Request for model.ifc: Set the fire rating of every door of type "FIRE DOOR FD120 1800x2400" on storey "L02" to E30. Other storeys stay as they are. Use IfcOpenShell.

First a look at what the model holds.

```python
import ifcopenshell
import ifcopenshell.util.element

model = ifcopenshell.open("model.ifc")
print(model.schema)
storey = next(s for s in model.by_type("IfcBuildingStorey") if s.Name == "L02")
doors = [e for e in ifcopenshell.util.element.get_decomposition(storey) if e.is_a("IfcDoor")]
seen = {}
for e in doors:
    element_type = ifcopenshell.util.element.get_type(e)
    key = (element_type.Name if element_type != e and element_type else None, ifcopenshell.util.element.get_pset(e, "Pset_DoorCommon", "FireRating"))
    seen[key] = seen.get(key, 0) + 1
for (name, value), count in sorted(seen.items(), key=str):
    print(count, "x", name, "|", value)
```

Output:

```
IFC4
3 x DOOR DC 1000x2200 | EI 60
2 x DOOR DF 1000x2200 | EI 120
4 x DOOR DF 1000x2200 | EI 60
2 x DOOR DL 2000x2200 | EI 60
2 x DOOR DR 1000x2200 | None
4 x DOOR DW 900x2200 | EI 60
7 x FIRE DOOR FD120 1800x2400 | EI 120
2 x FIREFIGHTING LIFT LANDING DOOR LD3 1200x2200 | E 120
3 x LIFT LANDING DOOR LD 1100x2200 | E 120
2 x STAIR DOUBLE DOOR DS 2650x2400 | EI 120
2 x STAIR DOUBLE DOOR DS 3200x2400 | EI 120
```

```python
import ifcopenshell
import ifcopenshell.api.pset
import ifcopenshell.util.element

model = ifcopenshell.open("model.ifc")

storey = next(s for s in model.by_type("IfcBuildingStorey") if s.Name == "L02")
doors = [e for e in ifcopenshell.util.element.get_decomposition(storey) if e.is_a("IfcDoor")]

count = 0
for e in doors:
    element_type = ifcopenshell.util.element.get_type(e)
    if element_type in (None, e) or element_type.Name != "FIRE DOOR FD120 1800x2400":
        continue
    found = ifcopenshell.util.element.get_pset(e, "Pset_DoorCommon", should_inherit=False)
    if found:
        pset = model.by_id(found["id"])
        if len(ifcopenshell.util.element.get_elements_by_pset(pset)) > 1:
            pset = ifcopenshell.api.pset.unshare_pset(model, products=[e], pset=pset)[0]
    else:
        pset = ifcopenshell.api.pset.add_pset(model, product=e, name="Pset_DoorCommon")
    ifcopenshell.api.pset.edit_pset(model, pset=pset, properties={"FireRating": "E30"})
    count += 1

print(count, "doors updated")

model.write("model_updated.ifc")
```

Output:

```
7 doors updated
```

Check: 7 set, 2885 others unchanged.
